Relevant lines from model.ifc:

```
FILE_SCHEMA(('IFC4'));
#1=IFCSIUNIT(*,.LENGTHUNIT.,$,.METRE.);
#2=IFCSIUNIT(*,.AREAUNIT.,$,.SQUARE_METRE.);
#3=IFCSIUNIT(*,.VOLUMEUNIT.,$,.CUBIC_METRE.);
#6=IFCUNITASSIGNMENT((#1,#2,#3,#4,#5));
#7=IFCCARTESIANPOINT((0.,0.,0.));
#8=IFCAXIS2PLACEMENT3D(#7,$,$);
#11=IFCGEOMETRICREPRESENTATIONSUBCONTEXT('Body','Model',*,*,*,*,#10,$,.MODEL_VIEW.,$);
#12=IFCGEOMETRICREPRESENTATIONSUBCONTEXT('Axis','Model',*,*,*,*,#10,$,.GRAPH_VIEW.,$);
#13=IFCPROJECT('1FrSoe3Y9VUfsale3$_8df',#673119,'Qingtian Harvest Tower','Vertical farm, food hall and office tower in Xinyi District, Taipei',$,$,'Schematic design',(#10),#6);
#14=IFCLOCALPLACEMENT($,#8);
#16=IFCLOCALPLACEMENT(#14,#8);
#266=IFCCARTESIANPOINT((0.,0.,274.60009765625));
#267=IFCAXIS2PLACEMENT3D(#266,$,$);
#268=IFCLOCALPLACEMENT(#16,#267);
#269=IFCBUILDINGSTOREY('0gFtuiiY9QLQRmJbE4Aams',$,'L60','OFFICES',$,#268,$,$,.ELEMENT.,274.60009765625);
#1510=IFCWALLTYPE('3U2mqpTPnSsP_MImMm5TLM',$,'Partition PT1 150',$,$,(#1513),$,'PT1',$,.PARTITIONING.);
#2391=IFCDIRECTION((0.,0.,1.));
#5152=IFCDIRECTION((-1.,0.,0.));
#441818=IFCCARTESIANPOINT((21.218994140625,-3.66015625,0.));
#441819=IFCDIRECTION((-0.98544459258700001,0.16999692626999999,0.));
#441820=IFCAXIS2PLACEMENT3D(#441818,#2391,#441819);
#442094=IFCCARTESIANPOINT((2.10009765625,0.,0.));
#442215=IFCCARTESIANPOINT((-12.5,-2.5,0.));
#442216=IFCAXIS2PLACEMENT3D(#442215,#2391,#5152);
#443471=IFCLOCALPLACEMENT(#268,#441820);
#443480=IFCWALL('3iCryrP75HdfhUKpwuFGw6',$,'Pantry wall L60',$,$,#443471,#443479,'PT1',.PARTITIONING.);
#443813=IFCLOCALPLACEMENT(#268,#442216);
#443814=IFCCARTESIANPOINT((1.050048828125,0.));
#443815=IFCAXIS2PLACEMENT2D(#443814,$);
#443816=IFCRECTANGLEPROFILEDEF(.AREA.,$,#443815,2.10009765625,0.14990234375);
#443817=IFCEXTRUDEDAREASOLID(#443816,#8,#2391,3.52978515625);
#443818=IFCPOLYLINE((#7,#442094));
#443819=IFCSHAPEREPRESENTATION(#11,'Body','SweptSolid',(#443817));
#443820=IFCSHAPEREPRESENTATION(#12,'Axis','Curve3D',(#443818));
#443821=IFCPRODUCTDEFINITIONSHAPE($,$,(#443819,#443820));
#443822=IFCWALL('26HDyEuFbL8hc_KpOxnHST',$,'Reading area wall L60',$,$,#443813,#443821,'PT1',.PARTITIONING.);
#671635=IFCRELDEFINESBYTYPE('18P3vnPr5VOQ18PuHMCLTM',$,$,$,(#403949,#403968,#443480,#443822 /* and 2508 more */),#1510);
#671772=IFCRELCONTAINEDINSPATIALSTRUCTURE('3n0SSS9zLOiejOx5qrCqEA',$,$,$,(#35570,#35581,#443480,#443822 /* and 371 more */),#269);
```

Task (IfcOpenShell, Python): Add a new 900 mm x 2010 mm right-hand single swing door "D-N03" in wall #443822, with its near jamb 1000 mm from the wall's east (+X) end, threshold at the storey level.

```python
import numpy as np
import ifcopenshell
import ifcopenshell.api.feature
import ifcopenshell.api.geometry
import ifcopenshell.api.root
import ifcopenshell.api.spatial
import ifcopenshell.geom
import ifcopenshell.util.element
import ifcopenshell.util.placement
import ifcopenshell.util.representation
import ifcopenshell.util.shape
import ifcopenshell.util.unit

model = ifcopenshell.open("model.ifc")
unit_scale = ifcopenshell.util.unit.calculate_unit_scale(model)
settings = ifcopenshell.geom.settings()


def volume(element):
    """Net volume in cubic metres, openings subtracted."""
    shape = ifcopenshell.geom.create_shape(settings, element)
    return ifcopenshell.util.shape.get_volume(shape.geometry)


wall = model.by_guid("26HDyEuFbL8hc_KpOxnHST")
storey = ifcopenshell.util.element.get_container(wall, ifc_class="IfcBuildingStorey")
context = ifcopenshell.util.representation.get_context(model, "Model", "Body", "MODEL_VIEW")
before = volume(wall)

width, height, from_end, sill = 0.9, 2.01, 1, 0.0  # metres

# The wall runs along its own X axis, and the end named is its -X end.
wall_shape = ifcopenshell.geom.create_shape(settings, wall)
x, y, z = ifcopenshell.util.shape.get_vertices(wall_shape.geometry).T
start = x.min() + from_end
face, thickness = float(y.min()), float(y.max() - y.min())
wall_matrix = ifcopenshell.util.placement.get_local_placement(wall.ObjectPlacement)
level = ifcopenshell.util.placement.get_local_placement(storey.ObjectPlacement)[2, 3]


def in_wall(x, y):
    """Placement at x, y metres in the wall's axes, at sill height."""
    matrix = wall_matrix.copy()
    matrix[:, 3] = wall_matrix @ np.array([x / unit_scale, y / unit_scale, 0.0, 1.0])
    matrix[2, 3] = level + sill / unit_scale
    return matrix


# Opening: a box that overshoots both wall faces by 50 mm.
opening = ifcopenshell.api.root.create_entity(model, ifc_class="IfcOpeningElement", predefined_type="OPENING")
box = ifcopenshell.api.geometry.add_wall_representation(
    model, context=context, length=width, height=height, thickness=thickness + 0.1
)
ifcopenshell.api.geometry.assign_representation(model, product=opening, representation=box)
ifcopenshell.api.geometry.edit_object_placement(model, product=opening, matrix=in_wall(start, face - 0.05), is_si=False)
ifcopenshell.api.feature.add_feature(model, feature=opening, element=wall)

door = ifcopenshell.api.root.create_entity(model, ifc_class="IfcDoor", name="D-N03", predefined_type="DOOR")
door.OverallWidth, door.OverallHeight = width / unit_scale, height / unit_scale
door.OperationType = "SINGLE_SWING_RIGHT"
body = ifcopenshell.api.geometry.add_door_representation(
    model,
    context=context,
    overall_width=door.OverallWidth,
    overall_height=door.OverallHeight,
    operation_type="SINGLE_SWING_RIGHT",
    lining_properties={"LiningDepth": thickness / unit_scale, "ThresholdDepth": thickness / unit_scale},
)
ifcopenshell.api.geometry.assign_representation(model, product=door, representation=body)
ifcopenshell.api.spatial.assign_container(model, products=[door], relating_structure=storey)
ifcopenshell.api.feature.add_filling(model, opening=opening, element=door)

# The lining spans the wall, so the door starts at the wall face.
ifcopenshell.api.geometry.edit_object_placement(model, product=door, matrix=in_wall(start, face), is_si=False)

after = volume(wall)

print(f"wall volume {before:.3f} -> {after:.3f} m3")

model.write("model_rev.ifc")
```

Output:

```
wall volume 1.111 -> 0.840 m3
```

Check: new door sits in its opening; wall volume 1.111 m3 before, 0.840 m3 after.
